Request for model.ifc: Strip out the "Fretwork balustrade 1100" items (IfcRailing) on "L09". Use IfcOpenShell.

First a look at what the model holds.

```python
import ifcopenshell
import ifcopenshell.util.element

model = ifcopenshell.open("model.ifc")
print(model.schema)
storey = next(s for s in model.by_type("IfcBuildingStorey") if s.Name == "L09")
railings = [e for e in ifcopenshell.util.element.get_decomposition(storey) if e.is_a("IfcRailing")]
seen = {}
for e in railings:
    element_type = ifcopenshell.util.element.get_type(e)
    name = element_type.Name if element_type not in (None, e) else None
    seen[name] = seen.get(name, 0) + 1
for name, count in sorted(seen.items(), key=str):
    print(count, "x", name)
```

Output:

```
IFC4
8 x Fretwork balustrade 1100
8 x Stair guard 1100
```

```python
import ifcopenshell
import ifcopenshell.api.root
import ifcopenshell.util.element

model = ifcopenshell.open("model.ifc")

storey = next(s for s in model.by_type("IfcBuildingStorey") if s.Name == "L09")
railings = [e for e in ifcopenshell.util.element.get_decomposition(storey) if e.is_a("IfcRailing")]
targets = [e for e in railings if (t := ifcopenshell.util.element.get_type(e)) not in (None, e) and t.Name == "Fretwork balustrade 1100"]

for e in targets:
    ifcopenshell.api.root.remove_product(model, product=e)
print(len(targets), "removed")

model.write("model_v2.ifc")
```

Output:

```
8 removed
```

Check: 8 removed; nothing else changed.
